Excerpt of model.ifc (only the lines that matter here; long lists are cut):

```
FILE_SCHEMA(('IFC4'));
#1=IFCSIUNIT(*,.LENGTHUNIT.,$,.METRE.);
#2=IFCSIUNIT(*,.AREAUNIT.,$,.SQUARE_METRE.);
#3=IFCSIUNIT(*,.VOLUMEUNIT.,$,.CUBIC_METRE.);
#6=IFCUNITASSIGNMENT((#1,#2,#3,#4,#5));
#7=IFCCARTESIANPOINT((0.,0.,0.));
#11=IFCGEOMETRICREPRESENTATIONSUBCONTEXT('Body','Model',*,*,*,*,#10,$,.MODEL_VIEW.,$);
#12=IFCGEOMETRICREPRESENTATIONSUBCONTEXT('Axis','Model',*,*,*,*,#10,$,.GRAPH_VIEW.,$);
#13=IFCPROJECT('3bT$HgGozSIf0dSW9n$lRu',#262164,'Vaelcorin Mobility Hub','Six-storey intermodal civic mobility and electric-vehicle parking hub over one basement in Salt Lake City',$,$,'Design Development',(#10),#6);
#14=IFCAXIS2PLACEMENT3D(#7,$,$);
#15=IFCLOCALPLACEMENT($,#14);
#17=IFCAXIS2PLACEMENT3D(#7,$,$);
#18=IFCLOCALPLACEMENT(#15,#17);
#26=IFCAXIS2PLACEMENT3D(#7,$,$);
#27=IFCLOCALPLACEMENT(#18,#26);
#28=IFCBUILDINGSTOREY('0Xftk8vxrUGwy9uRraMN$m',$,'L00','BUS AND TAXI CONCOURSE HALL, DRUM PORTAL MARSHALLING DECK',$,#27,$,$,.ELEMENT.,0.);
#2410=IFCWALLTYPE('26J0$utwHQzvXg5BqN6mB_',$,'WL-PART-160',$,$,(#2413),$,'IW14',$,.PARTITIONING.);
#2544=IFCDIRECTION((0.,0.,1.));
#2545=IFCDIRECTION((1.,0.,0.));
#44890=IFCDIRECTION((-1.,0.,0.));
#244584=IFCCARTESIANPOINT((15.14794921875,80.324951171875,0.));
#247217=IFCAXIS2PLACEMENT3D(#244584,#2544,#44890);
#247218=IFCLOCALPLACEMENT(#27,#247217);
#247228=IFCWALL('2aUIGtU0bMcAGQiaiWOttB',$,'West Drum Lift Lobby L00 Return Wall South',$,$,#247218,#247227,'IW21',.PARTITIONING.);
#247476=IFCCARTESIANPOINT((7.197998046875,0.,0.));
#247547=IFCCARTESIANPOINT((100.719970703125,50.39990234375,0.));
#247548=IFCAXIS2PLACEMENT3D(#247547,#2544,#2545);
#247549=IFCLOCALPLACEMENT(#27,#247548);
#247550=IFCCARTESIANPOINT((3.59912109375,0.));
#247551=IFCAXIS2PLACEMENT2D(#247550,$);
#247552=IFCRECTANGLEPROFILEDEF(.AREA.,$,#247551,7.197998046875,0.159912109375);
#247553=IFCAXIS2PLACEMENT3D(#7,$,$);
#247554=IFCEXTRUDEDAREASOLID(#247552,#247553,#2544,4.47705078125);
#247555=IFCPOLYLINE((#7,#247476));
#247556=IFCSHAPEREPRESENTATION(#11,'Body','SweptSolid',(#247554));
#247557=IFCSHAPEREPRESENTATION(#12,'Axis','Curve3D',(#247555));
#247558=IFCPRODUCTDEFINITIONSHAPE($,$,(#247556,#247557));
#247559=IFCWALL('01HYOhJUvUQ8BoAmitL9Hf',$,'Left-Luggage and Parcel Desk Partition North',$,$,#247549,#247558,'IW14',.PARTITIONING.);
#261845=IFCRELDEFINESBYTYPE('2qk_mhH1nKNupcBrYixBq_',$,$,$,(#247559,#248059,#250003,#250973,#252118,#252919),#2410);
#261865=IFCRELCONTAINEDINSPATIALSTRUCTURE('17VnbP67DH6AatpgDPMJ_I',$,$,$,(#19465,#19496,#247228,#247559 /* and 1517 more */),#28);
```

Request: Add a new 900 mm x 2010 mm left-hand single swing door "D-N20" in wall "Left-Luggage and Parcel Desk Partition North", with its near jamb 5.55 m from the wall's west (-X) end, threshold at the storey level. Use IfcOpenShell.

```python
import numpy as np
import ifcopenshell
import ifcopenshell.api.feature
import ifcopenshell.api.geometry
import ifcopenshell.api.root
import ifcopenshell.api.spatial
import ifcopenshell.geom
import ifcopenshell.util.element
import ifcopenshell.util.placement
import ifcopenshell.util.representation
import ifcopenshell.util.shape
import ifcopenshell.util.unit

model = ifcopenshell.open("model.ifc")
unit_scale = ifcopenshell.util.unit.calculate_unit_scale(model)
settings = ifcopenshell.geom.settings()


def volume(element):
    """Net volume in cubic metres, openings subtracted."""
    shape = ifcopenshell.geom.create_shape(settings, element)
    return ifcopenshell.util.shape.get_volume(shape.geometry)


wall = model.by_guid("01HYOhJUvUQ8BoAmitL9Hf")
storey = ifcopenshell.util.element.get_container(wall, ifc_class="IfcBuildingStorey")
context = ifcopenshell.util.representation.get_context(model, "Model", "Body", "MODEL_VIEW")
before = volume(wall)

width, height, from_end, sill = 0.9, 2.01, 5.55, 0.0  # metres

# The wall runs along its own X axis, and the end named is its -X end.
wall_shape = ifcopenshell.geom.create_shape(settings, wall)
x, y, z = ifcopenshell.util.shape.get_vertices(wall_shape.geometry).T
start = x.min() + from_end
face, thickness = float(y.min()), float(y.max() - y.min())
wall_matrix = ifcopenshell.util.placement.get_local_placement(wall.ObjectPlacement)
level = ifcopenshell.util.placement.get_local_placement(storey.ObjectPlacement)[2, 3]


def in_wall(x, y):
    """Placement at x, y metres in the wall's axes, at sill height."""
    matrix = wall_matrix.copy()
    matrix[:, 3] = wall_matrix @ np.array([x / unit_scale, y / unit_scale, 0.0, 1.0])
    matrix[2, 3] = level + sill / unit_scale
    return matrix


# Opening: a box that overshoots both wall faces by 50 mm.
opening = ifcopenshell.api.root.create_entity(model, ifc_class="IfcOpeningElement", predefined_type="OPENING")
box = ifcopenshell.api.geometry.add_wall_representation(
    model, context=context, length=width, height=height, thickness=thickness + 0.1
)
ifcopenshell.api.geometry.assign_representation(model, product=opening, representation=box)
ifcopenshell.api.geometry.edit_object_placement(model, product=opening, matrix=in_wall(start, face - 0.05), is_si=False)
ifcopenshell.api.feature.add_feature(model, feature=opening, element=wall)

door = ifcopenshell.api.root.create_entity(model, ifc_class="IfcDoor", name="D-N20", predefined_type="DOOR")
door.OverallWidth, door.OverallHeight = width / unit_scale, height / unit_scale
door.OperationType = "SINGLE_SWING_LEFT"
body = ifcopenshell.api.geometry.add_door_representation(
    model,
    context=context,
    overall_width=door.OverallWidth,
    overall_height=door.OverallHeight,
    operation_type="SINGLE_SWING_LEFT",
    lining_properties={"LiningDepth": thickness / unit_scale, "ThresholdDepth": thickness / unit_scale},
)
ifcopenshell.api.geometry.assign_representation(model, product=door, representation=body)
ifcopenshell.api.spatial.assign_container(model, products=[door], relating_structure=storey)
ifcopenshell.api.feature.add_filling(model, opening=opening, element=door)

# The lining spans the wall, so the door starts at the wall face.
ifcopenshell.api.geometry.edit_object_placement(model, product=door, matrix=in_wall(start, face), is_si=False)

after = volume(wall)

print(f"wall volume {before:.3f} -> {after:.3f} m3")

model.write("model_rev.ifc")
```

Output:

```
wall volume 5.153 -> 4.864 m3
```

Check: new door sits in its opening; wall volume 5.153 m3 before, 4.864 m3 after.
